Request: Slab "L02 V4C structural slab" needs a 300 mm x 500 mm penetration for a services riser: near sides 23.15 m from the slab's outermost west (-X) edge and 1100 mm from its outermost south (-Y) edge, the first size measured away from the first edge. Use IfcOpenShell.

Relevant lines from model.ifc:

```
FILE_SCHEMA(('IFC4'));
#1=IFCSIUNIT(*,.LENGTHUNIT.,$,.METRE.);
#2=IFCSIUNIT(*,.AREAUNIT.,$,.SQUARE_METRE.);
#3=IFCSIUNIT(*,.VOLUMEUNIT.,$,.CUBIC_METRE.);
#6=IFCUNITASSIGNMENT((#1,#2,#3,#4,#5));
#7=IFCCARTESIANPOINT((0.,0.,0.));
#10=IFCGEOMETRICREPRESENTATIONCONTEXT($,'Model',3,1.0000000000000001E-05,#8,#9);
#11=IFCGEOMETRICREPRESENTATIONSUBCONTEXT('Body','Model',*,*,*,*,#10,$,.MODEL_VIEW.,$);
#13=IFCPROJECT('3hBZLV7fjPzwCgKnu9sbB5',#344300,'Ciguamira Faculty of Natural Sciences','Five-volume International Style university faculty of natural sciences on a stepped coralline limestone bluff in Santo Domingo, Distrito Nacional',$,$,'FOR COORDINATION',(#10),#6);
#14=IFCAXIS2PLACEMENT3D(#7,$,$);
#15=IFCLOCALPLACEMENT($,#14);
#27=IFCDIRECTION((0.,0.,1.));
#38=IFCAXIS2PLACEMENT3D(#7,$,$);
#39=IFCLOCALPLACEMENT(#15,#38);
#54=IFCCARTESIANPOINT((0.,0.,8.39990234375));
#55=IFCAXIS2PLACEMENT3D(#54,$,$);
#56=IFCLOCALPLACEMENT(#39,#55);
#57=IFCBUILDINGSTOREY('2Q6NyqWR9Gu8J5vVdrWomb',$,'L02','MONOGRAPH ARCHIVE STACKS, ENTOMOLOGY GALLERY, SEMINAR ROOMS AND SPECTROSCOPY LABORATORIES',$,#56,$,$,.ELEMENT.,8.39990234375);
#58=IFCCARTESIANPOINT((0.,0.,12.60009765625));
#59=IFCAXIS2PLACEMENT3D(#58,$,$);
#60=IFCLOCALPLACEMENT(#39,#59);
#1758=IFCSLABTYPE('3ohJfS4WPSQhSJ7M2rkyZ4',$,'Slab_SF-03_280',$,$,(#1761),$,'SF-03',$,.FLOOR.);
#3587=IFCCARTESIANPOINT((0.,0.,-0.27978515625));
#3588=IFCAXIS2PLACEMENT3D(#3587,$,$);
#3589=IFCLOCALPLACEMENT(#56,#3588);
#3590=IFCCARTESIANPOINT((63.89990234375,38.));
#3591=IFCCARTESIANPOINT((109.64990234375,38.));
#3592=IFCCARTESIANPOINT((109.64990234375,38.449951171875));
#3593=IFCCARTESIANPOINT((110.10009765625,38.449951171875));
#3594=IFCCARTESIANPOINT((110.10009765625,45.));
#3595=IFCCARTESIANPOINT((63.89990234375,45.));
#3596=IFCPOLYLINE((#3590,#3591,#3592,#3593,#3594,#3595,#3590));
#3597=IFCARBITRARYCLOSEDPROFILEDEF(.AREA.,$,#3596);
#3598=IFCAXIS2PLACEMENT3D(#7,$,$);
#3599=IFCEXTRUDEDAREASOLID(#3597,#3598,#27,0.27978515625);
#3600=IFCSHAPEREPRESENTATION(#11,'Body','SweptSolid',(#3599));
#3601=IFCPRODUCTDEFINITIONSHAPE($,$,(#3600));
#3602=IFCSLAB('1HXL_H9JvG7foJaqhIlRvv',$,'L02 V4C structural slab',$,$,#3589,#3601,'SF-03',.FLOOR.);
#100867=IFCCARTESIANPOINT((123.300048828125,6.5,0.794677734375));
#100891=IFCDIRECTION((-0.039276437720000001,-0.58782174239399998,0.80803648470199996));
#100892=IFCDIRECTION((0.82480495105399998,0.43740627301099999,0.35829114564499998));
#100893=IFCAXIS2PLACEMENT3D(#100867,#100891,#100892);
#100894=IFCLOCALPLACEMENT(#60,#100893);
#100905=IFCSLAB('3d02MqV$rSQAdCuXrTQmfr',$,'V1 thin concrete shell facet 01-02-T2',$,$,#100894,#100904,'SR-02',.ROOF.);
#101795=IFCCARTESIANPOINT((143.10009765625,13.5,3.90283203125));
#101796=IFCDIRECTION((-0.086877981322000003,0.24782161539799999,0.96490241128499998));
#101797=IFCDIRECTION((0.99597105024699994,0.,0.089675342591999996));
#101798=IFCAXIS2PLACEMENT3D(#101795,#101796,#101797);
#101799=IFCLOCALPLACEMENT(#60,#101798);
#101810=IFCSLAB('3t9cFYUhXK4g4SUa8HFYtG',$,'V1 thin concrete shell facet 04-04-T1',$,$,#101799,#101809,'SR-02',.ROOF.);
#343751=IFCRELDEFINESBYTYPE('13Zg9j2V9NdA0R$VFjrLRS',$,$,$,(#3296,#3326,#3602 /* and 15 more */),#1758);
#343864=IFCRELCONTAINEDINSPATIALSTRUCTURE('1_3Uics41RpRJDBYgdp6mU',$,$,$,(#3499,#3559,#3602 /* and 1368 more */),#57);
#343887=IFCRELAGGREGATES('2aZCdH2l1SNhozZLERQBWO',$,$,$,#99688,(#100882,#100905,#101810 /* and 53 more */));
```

```python
import numpy as np
import ifcopenshell
import ifcopenshell.api.feature
import ifcopenshell.api.geometry
import ifcopenshell.api.root
import ifcopenshell.geom
import ifcopenshell.util.placement
import ifcopenshell.util.representation
import ifcopenshell.util.shape
import ifcopenshell.util.unit

model = ifcopenshell.open("model.ifc")
unit_scale = ifcopenshell.util.unit.calculate_unit_scale(model)
settings = ifcopenshell.geom.settings()


def volume(element):
    """Net volume in cubic metres, openings subtracted."""
    shape = ifcopenshell.geom.create_shape(settings, element)
    return ifcopenshell.util.shape.get_volume(shape.geometry)


slab = model.by_guid("1HXL_H9JvG7foJaqhIlRvv")
before = volume(slab)

# Extent in the slab's own axes, in metres. The edges named are its -X and -Y sides.
slab_shape = ifcopenshell.geom.create_shape(settings, slab)
vertices = ifcopenshell.util.shape.get_vertices(slab_shape.geometry)
x_min, y_min, bottom = vertices.min(axis=0)
top = vertices[:, 2].max()

opening = ifcopenshell.api.root.create_entity(model, ifc_class="IfcOpeningElement", name="Services riser opening", predefined_type="OPENING")
context = ifcopenshell.util.representation.get_context(model, "Model", "Body", "MODEL_VIEW")
width, depth = 0.3, 0.5
outline = [(0.0, 0.0), (width, 0.0), (width, depth), (0.0, depth), (0.0, 0.0)]
# Overshoot both faces by 50 mm so the cut is clean.
shape = ifcopenshell.api.geometry.add_slab_representation(
    model, context=context, depth=top - bottom + 0.1, polyline=outline
)
ifcopenshell.api.geometry.assign_representation(model, product=opening, representation=shape)

matrix = ifcopenshell.util.placement.get_local_placement(slab.ObjectPlacement)
matrix[:, 3] = matrix @ np.append(np.array([x_min + 23.15, y_min + 1.1, bottom - 0.05]) / unit_scale, 1.0)
ifcopenshell.api.geometry.edit_object_placement(model, product=opening, matrix=matrix, is_si=False)
ifcopenshell.api.feature.add_feature(model, feature=opening, element=slab)

after = volume(slab)

print(f"slab volume {before:.3f} -> {after:.3f} m3")

model.write("model_rev.ifc")
```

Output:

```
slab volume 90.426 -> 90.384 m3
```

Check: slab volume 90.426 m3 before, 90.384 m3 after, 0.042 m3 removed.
